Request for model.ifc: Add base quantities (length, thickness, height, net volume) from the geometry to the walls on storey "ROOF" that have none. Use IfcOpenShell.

First a look at what the model holds.

```python
import ifcopenshell
import ifcopenshell.util.element
import ifcopenshell.util.unit

model = ifcopenshell.open("model.ifc")
print(model.schema)
for unit_type in ("LENGTHUNIT", "AREAUNIT", "VOLUMEUNIT"):
    print(unit_type, ifcopenshell.util.unit.calculate_unit_scale(model, unit_type))
storey = next(s for s in model.by_type("IfcBuildingStorey") if s.Name == "ROOF")
walls = [e for e in ifcopenshell.util.element.get_decomposition(storey) if e.is_a("IfcWall")]
for e in sorted(walls, key=lambda e: e.id()):
    print(e.id(), e.is_a(), e.Name, list(ifcopenshell.util.element.get_psets(e, qtos_only=True)), sep=" | ")
```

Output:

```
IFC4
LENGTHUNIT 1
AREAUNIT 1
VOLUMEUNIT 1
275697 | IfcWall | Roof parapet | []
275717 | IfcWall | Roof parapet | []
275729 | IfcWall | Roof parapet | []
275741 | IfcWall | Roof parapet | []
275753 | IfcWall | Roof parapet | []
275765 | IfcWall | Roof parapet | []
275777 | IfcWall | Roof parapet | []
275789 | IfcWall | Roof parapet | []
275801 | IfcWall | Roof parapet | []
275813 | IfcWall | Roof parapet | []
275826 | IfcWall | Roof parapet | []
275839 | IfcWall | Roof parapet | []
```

```python
import ifcopenshell
import ifcopenshell.api.pset
import ifcopenshell.geom
import ifcopenshell.util.element
import ifcopenshell.util.shape
import ifcopenshell.util.unit

model = ifcopenshell.open("model.ifc")
unit_scale = ifcopenshell.util.unit.calculate_unit_scale(model)
volume_scale = ifcopenshell.util.unit.calculate_unit_scale(model, "VOLUMEUNIT")
settings = ifcopenshell.geom.settings()

storey = next(s for s in model.by_type("IfcBuildingStorey") if s.Name == "ROOF")
walls = [e for e in ifcopenshell.util.element.get_decomposition(storey) if e.is_a("IfcWall")]

for e in sorted(walls, key=lambda e: e.id()):
    if ifcopenshell.util.element.get_psets(e, qtos_only=True, should_inherit=False):
        continue
    # Geometry comes back in metres, in the element's own axes.
    shape = ifcopenshell.geom.create_shape(settings, e)
    values = {
        "Length": ifcopenshell.util.shape.get_x(shape.geometry) / unit_scale,
        "Width": ifcopenshell.util.shape.get_y(shape.geometry) / unit_scale,
        "Height": ifcopenshell.util.shape.get_z(shape.geometry) / unit_scale,
        "NetVolume": ifcopenshell.util.shape.get_volume(shape.geometry) / volume_scale,
    }
    qto = ifcopenshell.api.pset.add_qto(model, product=e, name="Qto_WallBaseQuantities")
    ifcopenshell.api.pset.edit_qto(model, qto=qto, properties=values)
    print(e.id(), {k: round(v, 3) for k, v in values.items()})

model.write("model_rev.ifc")
```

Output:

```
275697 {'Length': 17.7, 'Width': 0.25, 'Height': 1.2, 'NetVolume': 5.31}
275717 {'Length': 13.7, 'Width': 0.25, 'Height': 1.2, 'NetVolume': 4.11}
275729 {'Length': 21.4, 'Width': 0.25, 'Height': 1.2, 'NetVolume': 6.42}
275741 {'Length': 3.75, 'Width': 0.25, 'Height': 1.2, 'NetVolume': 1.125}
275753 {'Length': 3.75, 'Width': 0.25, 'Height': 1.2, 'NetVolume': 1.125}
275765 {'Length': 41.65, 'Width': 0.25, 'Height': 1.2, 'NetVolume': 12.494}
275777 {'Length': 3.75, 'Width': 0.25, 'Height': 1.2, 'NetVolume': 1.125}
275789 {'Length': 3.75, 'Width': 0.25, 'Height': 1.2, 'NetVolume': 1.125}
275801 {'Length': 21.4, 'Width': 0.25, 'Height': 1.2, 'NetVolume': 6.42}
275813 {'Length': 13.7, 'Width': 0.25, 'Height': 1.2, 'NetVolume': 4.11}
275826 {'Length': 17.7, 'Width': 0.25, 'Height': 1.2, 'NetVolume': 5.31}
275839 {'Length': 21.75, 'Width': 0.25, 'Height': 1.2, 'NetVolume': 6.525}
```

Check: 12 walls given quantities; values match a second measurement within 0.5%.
